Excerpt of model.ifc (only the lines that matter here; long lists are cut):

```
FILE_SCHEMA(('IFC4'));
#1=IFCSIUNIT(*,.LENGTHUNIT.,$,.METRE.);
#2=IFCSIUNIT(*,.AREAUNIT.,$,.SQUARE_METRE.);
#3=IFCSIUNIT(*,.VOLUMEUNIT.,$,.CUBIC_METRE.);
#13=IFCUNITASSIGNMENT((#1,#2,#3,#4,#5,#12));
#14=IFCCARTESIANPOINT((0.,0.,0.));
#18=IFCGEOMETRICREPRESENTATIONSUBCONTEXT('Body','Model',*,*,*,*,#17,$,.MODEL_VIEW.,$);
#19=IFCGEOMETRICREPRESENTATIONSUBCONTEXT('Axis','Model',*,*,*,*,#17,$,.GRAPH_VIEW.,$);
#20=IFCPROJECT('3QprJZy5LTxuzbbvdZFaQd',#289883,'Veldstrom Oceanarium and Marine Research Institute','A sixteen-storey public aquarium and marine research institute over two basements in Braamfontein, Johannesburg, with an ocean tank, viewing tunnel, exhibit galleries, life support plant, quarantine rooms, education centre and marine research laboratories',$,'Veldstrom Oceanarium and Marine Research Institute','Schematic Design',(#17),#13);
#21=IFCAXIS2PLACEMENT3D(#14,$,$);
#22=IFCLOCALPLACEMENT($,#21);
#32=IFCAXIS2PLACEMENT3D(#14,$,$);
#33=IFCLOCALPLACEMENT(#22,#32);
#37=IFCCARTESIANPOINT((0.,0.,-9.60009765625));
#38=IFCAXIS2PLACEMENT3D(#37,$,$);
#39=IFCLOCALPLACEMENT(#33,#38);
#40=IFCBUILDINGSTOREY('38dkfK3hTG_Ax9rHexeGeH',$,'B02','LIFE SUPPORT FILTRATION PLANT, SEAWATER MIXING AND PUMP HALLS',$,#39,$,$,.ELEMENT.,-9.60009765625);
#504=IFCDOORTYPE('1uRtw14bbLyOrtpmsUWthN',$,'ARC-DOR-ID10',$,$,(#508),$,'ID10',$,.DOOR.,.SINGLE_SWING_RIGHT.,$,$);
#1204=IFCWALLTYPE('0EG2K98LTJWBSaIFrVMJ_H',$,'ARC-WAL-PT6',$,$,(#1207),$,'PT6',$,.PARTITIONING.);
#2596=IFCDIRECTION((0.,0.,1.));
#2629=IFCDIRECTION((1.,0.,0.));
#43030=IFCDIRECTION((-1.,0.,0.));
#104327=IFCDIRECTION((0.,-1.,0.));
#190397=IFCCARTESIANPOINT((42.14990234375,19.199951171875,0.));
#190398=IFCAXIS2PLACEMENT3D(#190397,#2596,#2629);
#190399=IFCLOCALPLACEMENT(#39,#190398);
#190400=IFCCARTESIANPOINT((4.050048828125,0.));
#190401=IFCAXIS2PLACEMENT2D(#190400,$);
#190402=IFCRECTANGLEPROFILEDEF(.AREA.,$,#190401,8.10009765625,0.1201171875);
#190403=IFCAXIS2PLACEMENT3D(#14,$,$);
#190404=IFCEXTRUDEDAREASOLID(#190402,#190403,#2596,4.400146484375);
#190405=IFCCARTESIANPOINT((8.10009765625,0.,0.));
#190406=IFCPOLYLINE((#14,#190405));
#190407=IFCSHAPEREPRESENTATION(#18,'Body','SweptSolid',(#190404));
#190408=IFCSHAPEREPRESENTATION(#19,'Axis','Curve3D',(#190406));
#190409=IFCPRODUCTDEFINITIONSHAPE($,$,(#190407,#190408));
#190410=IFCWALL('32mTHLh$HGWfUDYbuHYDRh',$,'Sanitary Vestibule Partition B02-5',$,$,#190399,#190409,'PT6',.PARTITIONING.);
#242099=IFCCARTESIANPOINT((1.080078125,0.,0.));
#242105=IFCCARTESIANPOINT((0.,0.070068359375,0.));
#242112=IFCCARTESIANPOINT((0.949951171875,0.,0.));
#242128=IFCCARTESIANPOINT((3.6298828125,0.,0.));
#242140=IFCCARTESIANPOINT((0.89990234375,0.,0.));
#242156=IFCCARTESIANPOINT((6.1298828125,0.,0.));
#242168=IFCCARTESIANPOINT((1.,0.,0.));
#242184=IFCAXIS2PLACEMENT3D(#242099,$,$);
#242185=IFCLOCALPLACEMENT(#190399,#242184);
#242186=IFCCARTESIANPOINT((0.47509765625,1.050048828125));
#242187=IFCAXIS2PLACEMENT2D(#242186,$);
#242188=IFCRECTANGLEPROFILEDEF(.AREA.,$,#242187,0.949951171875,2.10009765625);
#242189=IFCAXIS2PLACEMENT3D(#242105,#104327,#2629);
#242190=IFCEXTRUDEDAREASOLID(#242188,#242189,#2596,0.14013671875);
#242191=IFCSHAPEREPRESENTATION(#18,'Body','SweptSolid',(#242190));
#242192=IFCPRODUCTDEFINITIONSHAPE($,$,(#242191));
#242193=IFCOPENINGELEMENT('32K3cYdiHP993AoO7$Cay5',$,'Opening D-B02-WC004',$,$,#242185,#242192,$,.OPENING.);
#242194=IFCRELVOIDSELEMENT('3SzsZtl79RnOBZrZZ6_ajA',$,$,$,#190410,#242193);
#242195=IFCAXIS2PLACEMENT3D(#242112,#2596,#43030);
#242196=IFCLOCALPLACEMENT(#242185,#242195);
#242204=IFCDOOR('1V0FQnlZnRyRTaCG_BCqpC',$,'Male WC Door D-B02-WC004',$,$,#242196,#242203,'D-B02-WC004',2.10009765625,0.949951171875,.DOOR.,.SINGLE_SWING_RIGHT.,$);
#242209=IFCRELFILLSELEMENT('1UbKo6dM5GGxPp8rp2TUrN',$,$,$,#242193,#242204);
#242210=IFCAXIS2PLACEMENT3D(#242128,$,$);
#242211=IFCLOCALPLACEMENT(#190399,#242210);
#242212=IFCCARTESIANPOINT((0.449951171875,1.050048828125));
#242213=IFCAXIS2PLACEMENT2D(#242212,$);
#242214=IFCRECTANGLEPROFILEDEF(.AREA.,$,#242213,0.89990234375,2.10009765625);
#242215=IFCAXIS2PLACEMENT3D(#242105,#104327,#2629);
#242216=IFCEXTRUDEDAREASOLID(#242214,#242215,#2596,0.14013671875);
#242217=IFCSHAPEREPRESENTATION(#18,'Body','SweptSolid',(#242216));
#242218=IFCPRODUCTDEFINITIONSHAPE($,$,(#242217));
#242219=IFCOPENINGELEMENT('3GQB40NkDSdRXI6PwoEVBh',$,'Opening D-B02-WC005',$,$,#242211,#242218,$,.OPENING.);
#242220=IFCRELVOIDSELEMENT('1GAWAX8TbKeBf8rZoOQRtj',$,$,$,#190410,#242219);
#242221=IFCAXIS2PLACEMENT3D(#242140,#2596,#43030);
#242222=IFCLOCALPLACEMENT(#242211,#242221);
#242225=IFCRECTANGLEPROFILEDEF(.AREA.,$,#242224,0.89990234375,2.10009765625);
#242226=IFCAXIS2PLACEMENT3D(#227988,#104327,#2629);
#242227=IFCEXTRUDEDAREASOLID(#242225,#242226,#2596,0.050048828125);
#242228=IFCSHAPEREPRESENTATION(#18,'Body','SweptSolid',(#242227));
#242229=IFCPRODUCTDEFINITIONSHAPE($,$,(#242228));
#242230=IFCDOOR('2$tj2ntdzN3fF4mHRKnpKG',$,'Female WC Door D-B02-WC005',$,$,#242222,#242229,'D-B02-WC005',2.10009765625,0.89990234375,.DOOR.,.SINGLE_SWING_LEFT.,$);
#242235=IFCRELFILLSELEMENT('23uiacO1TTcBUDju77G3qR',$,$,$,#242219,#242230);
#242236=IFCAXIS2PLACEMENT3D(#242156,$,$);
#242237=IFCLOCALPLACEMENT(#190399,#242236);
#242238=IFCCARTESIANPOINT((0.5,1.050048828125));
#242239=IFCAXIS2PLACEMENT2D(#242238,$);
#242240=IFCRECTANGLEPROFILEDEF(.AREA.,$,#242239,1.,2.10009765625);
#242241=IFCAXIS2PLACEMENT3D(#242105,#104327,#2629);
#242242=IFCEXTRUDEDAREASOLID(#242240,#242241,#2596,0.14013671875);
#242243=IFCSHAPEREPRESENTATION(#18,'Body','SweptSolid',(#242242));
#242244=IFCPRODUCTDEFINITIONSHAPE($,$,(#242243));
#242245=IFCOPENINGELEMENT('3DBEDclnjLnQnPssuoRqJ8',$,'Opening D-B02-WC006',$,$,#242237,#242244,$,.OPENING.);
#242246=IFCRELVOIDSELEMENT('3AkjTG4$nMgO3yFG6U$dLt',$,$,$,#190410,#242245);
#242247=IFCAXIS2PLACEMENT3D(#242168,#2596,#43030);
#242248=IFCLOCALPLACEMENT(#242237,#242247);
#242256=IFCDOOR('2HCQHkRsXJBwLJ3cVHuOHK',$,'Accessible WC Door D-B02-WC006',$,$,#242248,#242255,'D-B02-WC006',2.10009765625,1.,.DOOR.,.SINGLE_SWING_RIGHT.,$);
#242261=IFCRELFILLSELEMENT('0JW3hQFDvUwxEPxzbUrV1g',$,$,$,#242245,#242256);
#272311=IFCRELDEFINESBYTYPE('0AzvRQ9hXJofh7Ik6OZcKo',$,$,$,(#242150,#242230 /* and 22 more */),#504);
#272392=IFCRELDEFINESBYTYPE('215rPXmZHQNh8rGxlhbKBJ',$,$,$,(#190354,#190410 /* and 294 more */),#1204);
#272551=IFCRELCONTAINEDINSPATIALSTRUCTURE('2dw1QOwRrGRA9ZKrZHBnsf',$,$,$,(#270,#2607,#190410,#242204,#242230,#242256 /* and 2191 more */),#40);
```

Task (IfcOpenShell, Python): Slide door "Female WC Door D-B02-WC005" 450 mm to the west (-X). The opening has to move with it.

```python
import ifcopenshell
import ifcopenshell.api.geometry
import ifcopenshell.util.placement
import ifcopenshell.util.unit

model = ifcopenshell.open("model.ifc")
unit_scale = ifcopenshell.util.unit.calculate_unit_scale(model)

door = model.by_id(242230)
opening = door.FillsVoids[0].RelatingOpeningElement
wall = opening.VoidsElements[0].RelatingBuildingElement

wall_matrix = ifcopenshell.util.placement.get_local_placement(wall.ObjectPlacement)
shift = wall_matrix[:3, 0] * -0.45 / unit_scale
before = ifcopenshell.util.placement.get_local_placement(door.ObjectPlacement)[:3, 3].copy()

# The door is placed relative to its opening, so it follows when the opening moves.
matrix = ifcopenshell.util.placement.get_local_placement(opening.ObjectPlacement)
matrix[:3, 3] += shift
ifcopenshell.api.geometry.edit_object_placement(
    model, product=opening, matrix=matrix, is_si=False, should_transform_children=True
)

after = ifcopenshell.util.placement.get_local_placement(door.ObjectPlacement)[:3, 3]
print("door moved by", (after - before).round(3) + 0.0)

model.write("model_updated.ifc")
```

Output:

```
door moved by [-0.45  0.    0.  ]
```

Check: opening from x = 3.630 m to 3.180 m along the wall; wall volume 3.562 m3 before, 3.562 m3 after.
